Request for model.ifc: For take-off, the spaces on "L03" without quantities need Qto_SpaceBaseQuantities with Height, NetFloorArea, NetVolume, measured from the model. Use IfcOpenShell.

First a look at what the model holds.

```python
import ifcopenshell
import ifcopenshell.util.element
import ifcopenshell.util.unit

model = ifcopenshell.open("model.ifc")
print(model.schema)
for unit_type in ("LENGTHUNIT", "AREAUNIT", "VOLUMEUNIT"):
    print(unit_type, ifcopenshell.util.unit.calculate_unit_scale(model, unit_type))
storey = next(s for s in model.by_type("IfcBuildingStorey") if s.Name == "L03")
spaces = [e for e in ifcopenshell.util.element.get_decomposition(storey) if e.is_a("IfcSpace")]
for e in sorted(spaces, key=lambda e: e.id()):
    print(e.id(), e.is_a(), e.Name, list(ifcopenshell.util.element.get_psets(e, qtos_only=True)), sep=" | ")
```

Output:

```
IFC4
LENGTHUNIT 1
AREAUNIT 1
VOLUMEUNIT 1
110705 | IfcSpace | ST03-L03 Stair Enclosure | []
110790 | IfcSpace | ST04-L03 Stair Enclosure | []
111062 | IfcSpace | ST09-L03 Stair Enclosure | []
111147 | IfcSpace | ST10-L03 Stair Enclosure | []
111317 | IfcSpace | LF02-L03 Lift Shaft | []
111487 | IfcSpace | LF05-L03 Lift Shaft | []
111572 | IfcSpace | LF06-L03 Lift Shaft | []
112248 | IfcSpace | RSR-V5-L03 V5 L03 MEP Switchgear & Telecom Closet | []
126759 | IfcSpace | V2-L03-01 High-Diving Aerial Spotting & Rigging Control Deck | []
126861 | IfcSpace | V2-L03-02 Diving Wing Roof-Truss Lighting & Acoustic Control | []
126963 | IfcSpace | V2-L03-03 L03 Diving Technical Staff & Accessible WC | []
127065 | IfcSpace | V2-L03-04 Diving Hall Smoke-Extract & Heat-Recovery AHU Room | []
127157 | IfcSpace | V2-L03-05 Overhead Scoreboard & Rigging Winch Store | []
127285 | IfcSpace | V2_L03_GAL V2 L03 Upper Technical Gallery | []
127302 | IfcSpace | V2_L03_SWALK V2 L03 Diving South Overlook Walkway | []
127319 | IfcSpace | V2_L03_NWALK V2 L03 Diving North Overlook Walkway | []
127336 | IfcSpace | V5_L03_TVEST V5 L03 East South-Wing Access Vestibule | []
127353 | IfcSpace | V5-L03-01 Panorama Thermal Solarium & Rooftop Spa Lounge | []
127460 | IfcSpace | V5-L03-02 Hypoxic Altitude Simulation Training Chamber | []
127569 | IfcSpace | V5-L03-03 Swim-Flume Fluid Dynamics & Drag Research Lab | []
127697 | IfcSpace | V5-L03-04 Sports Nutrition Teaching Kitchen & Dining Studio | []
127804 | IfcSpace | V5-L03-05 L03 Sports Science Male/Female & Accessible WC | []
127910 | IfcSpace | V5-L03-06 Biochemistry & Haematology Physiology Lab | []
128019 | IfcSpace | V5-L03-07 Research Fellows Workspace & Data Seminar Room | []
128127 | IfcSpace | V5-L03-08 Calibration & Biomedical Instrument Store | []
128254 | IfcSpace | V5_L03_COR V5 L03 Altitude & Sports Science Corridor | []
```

```python
import ifcopenshell
import ifcopenshell.api.pset
import ifcopenshell.geom
import ifcopenshell.util.element
import ifcopenshell.util.shape
import ifcopenshell.util.unit

model = ifcopenshell.open("model.ifc")
unit_scale = ifcopenshell.util.unit.calculate_unit_scale(model)
area_scale = ifcopenshell.util.unit.calculate_unit_scale(model, "AREAUNIT")
volume_scale = ifcopenshell.util.unit.calculate_unit_scale(model, "VOLUMEUNIT")
settings = ifcopenshell.geom.settings()

storey = next(s for s in model.by_type("IfcBuildingStorey") if s.Name == "L03")
spaces = [e for e in ifcopenshell.util.element.get_decomposition(storey) if e.is_a("IfcSpace")]

for e in sorted(spaces, key=lambda e: e.id()):
    if ifcopenshell.util.element.get_psets(e, qtos_only=True, should_inherit=False):
        continue
    # Geometry comes back in metres, in the element's own axes.
    shape = ifcopenshell.geom.create_shape(settings, e)
    values = {
        "Height": ifcopenshell.util.shape.get_z(shape.geometry) / unit_scale,
        "NetFloorArea": ifcopenshell.util.shape.get_footprint_area(shape.geometry) / area_scale,
        "NetVolume": ifcopenshell.util.shape.get_volume(shape.geometry) / volume_scale,
    }
    qto = ifcopenshell.api.pset.add_qto(model, product=e, name="Qto_SpaceBaseQuantities")
    ifcopenshell.api.pset.edit_qto(model, qto=qto, properties=values)
    print(e.id(), {k: round(v, 3) for k, v in values.items()})

model.write("model_updated.ifc")
```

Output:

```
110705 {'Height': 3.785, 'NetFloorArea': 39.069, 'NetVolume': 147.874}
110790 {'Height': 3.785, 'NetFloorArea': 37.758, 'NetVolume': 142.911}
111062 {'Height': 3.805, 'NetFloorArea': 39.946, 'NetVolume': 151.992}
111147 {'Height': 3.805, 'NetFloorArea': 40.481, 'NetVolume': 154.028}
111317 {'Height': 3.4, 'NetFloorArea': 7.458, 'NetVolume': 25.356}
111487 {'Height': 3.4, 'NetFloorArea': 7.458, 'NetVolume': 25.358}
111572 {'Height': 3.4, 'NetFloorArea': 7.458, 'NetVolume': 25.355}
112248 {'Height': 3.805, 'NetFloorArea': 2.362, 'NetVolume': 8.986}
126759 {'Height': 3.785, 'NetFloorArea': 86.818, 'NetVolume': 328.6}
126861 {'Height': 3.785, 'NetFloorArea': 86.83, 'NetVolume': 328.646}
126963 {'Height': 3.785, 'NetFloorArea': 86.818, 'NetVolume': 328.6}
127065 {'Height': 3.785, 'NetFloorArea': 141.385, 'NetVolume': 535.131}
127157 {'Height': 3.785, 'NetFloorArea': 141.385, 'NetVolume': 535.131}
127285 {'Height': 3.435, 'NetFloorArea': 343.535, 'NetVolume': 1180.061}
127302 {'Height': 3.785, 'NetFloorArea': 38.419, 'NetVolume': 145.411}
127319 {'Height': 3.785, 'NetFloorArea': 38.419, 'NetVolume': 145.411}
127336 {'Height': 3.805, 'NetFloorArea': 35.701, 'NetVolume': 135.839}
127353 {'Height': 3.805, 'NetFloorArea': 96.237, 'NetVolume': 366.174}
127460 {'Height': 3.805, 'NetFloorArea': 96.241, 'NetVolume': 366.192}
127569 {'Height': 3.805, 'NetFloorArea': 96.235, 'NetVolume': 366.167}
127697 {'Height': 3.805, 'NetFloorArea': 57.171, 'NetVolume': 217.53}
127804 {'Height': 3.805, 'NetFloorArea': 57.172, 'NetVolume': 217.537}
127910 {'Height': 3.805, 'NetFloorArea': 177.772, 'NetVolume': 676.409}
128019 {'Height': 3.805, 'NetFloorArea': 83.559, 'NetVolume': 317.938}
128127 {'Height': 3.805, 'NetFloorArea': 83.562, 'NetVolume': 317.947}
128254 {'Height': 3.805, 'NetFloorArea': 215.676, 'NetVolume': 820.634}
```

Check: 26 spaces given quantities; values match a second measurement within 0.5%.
